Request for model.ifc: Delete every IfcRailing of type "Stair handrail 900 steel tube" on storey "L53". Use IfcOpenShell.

First a look at what the model holds.

```python
import ifcopenshell
import ifcopenshell.util.element

model = ifcopenshell.open("model.ifc")
print(model.schema)
storey = next(s for s in model.by_type("IfcBuildingStorey") if s.Name == "L53")
railings = [e for e in ifcopenshell.util.element.get_decomposition(storey) if e.is_a("IfcRailing")]
seen = {}
for e in railings:
    element_type = ifcopenshell.util.element.get_type(e)
    name = element_type.Name if element_type not in (None, e) else None
    seen[name] = seen.get(name, 0) + 1
for name, count in sorted(seen.items(), key=str):
    print(count, "x", name)
```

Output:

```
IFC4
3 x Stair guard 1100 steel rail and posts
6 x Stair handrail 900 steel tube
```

```python
import ifcopenshell
import ifcopenshell.api.root
import ifcopenshell.util.element

model = ifcopenshell.open("model.ifc")

storey = next(s for s in model.by_type("IfcBuildingStorey") if s.Name == "L53")
railings = [e for e in ifcopenshell.util.element.get_decomposition(storey) if e.is_a("IfcRailing")]
targets = [e for e in railings if (t := ifcopenshell.util.element.get_type(e)) not in (None, e) and t.Name == "Stair handrail 900 steel tube"]

for e in targets:
    ifcopenshell.api.root.remove_product(model, product=e)
print(len(targets), "removed")

model.write("model_updated.ifc")
```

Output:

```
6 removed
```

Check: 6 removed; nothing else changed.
